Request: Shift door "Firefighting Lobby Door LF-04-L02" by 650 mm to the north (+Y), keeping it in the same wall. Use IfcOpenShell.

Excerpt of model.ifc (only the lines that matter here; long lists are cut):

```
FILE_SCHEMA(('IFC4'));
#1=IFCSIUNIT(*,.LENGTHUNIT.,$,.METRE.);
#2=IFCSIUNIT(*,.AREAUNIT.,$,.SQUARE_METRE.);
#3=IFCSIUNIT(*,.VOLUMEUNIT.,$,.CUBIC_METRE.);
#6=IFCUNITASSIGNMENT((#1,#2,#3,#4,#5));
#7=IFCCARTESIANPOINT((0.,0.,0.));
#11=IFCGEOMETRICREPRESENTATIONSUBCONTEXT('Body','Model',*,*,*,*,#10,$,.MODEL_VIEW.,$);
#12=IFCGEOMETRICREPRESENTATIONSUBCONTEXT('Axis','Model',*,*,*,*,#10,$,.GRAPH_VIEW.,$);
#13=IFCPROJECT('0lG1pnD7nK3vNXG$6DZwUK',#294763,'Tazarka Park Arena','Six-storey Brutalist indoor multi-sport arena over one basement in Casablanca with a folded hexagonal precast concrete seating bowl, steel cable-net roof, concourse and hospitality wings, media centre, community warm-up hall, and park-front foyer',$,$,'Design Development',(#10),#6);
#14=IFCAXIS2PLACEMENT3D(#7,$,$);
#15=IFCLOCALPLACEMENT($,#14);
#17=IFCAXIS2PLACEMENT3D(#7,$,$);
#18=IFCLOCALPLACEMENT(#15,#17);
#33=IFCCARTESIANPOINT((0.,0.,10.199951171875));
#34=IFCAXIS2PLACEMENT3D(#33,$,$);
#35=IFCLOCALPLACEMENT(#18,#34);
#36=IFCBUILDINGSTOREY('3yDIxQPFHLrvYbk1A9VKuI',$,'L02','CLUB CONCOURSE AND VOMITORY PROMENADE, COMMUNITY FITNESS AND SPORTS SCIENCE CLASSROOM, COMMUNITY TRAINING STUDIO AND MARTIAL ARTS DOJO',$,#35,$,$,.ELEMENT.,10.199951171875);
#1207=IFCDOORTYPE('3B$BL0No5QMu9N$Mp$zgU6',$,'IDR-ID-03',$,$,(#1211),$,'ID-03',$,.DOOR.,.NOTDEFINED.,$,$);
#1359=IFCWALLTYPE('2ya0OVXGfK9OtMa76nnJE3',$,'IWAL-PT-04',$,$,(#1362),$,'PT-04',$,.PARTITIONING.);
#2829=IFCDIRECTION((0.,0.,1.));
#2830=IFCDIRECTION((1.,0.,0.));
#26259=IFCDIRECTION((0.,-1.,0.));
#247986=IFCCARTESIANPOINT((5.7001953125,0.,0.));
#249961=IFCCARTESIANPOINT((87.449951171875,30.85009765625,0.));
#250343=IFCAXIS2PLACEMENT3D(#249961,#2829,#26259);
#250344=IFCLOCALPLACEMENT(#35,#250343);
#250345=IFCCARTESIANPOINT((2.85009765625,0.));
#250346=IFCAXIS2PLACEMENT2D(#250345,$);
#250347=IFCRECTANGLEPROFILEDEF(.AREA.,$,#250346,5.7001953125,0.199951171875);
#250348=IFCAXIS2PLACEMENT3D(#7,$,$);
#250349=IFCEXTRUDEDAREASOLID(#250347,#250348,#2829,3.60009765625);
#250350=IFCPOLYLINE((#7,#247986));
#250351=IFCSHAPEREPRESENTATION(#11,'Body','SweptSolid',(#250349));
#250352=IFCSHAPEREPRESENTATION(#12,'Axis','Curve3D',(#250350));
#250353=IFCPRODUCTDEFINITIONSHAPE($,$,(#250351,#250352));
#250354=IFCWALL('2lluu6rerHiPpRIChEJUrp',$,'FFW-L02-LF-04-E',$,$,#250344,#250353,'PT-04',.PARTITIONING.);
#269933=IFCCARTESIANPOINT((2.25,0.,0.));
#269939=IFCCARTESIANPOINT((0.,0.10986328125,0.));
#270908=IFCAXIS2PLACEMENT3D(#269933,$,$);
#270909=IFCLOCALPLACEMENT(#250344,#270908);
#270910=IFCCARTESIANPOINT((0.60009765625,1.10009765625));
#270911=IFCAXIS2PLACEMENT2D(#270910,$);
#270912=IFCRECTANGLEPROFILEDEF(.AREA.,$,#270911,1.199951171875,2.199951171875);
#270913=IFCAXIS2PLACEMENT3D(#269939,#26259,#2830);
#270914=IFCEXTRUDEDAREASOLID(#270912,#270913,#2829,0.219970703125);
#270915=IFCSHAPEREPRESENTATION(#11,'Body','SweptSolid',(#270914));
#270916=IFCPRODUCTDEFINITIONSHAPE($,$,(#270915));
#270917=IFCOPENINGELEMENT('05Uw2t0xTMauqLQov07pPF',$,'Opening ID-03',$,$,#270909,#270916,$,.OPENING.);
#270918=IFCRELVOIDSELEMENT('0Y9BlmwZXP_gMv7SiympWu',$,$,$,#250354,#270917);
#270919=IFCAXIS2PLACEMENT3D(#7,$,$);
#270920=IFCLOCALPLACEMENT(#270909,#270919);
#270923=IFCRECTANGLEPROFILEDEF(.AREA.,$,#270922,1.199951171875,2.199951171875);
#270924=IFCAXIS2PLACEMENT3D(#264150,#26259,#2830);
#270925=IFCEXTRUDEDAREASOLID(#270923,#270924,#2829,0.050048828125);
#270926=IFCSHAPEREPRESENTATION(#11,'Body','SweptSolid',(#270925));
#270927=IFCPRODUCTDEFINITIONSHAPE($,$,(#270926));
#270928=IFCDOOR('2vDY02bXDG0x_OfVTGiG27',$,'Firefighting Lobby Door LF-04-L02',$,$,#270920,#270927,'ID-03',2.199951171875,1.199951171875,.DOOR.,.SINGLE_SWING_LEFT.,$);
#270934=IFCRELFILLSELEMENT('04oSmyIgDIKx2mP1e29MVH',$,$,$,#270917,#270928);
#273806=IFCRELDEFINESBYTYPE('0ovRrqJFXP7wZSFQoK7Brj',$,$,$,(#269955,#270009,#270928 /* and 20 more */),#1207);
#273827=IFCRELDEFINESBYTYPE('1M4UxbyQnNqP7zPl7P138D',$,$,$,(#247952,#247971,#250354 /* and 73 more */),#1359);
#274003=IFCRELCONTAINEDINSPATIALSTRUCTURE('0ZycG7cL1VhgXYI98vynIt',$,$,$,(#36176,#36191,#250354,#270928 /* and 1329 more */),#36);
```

```python
import ifcopenshell
import ifcopenshell.api.geometry
import ifcopenshell.util.placement

model = ifcopenshell.open("model.ifc")

door = model.by_id(270928)
opening = door.FillsVoids[0].RelatingOpeningElement
wall = opening.VoidsElements[0].RelatingBuildingElement

wall_matrix = ifcopenshell.util.placement.get_local_placement(wall.ObjectPlacement)
shift = wall_matrix[:3, 0] * -0.65
before = ifcopenshell.util.placement.get_local_placement(door.ObjectPlacement)[:3, 3].copy()

# The door is placed relative to its opening, so it follows when the opening moves.
matrix = ifcopenshell.util.placement.get_local_placement(opening.ObjectPlacement)
matrix[:3, 3] += shift
ifcopenshell.api.geometry.edit_object_placement(
    model, product=opening, matrix=matrix, is_si=False, should_transform_children=True
)

after = ifcopenshell.util.placement.get_local_placement(door.ObjectPlacement)[:3, 3]
print("door moved by", (after - before).round(3) + 0.0)

model.write("model-out.ifc")
```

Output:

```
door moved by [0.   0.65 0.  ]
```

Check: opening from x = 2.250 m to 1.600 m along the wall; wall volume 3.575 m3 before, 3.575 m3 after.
